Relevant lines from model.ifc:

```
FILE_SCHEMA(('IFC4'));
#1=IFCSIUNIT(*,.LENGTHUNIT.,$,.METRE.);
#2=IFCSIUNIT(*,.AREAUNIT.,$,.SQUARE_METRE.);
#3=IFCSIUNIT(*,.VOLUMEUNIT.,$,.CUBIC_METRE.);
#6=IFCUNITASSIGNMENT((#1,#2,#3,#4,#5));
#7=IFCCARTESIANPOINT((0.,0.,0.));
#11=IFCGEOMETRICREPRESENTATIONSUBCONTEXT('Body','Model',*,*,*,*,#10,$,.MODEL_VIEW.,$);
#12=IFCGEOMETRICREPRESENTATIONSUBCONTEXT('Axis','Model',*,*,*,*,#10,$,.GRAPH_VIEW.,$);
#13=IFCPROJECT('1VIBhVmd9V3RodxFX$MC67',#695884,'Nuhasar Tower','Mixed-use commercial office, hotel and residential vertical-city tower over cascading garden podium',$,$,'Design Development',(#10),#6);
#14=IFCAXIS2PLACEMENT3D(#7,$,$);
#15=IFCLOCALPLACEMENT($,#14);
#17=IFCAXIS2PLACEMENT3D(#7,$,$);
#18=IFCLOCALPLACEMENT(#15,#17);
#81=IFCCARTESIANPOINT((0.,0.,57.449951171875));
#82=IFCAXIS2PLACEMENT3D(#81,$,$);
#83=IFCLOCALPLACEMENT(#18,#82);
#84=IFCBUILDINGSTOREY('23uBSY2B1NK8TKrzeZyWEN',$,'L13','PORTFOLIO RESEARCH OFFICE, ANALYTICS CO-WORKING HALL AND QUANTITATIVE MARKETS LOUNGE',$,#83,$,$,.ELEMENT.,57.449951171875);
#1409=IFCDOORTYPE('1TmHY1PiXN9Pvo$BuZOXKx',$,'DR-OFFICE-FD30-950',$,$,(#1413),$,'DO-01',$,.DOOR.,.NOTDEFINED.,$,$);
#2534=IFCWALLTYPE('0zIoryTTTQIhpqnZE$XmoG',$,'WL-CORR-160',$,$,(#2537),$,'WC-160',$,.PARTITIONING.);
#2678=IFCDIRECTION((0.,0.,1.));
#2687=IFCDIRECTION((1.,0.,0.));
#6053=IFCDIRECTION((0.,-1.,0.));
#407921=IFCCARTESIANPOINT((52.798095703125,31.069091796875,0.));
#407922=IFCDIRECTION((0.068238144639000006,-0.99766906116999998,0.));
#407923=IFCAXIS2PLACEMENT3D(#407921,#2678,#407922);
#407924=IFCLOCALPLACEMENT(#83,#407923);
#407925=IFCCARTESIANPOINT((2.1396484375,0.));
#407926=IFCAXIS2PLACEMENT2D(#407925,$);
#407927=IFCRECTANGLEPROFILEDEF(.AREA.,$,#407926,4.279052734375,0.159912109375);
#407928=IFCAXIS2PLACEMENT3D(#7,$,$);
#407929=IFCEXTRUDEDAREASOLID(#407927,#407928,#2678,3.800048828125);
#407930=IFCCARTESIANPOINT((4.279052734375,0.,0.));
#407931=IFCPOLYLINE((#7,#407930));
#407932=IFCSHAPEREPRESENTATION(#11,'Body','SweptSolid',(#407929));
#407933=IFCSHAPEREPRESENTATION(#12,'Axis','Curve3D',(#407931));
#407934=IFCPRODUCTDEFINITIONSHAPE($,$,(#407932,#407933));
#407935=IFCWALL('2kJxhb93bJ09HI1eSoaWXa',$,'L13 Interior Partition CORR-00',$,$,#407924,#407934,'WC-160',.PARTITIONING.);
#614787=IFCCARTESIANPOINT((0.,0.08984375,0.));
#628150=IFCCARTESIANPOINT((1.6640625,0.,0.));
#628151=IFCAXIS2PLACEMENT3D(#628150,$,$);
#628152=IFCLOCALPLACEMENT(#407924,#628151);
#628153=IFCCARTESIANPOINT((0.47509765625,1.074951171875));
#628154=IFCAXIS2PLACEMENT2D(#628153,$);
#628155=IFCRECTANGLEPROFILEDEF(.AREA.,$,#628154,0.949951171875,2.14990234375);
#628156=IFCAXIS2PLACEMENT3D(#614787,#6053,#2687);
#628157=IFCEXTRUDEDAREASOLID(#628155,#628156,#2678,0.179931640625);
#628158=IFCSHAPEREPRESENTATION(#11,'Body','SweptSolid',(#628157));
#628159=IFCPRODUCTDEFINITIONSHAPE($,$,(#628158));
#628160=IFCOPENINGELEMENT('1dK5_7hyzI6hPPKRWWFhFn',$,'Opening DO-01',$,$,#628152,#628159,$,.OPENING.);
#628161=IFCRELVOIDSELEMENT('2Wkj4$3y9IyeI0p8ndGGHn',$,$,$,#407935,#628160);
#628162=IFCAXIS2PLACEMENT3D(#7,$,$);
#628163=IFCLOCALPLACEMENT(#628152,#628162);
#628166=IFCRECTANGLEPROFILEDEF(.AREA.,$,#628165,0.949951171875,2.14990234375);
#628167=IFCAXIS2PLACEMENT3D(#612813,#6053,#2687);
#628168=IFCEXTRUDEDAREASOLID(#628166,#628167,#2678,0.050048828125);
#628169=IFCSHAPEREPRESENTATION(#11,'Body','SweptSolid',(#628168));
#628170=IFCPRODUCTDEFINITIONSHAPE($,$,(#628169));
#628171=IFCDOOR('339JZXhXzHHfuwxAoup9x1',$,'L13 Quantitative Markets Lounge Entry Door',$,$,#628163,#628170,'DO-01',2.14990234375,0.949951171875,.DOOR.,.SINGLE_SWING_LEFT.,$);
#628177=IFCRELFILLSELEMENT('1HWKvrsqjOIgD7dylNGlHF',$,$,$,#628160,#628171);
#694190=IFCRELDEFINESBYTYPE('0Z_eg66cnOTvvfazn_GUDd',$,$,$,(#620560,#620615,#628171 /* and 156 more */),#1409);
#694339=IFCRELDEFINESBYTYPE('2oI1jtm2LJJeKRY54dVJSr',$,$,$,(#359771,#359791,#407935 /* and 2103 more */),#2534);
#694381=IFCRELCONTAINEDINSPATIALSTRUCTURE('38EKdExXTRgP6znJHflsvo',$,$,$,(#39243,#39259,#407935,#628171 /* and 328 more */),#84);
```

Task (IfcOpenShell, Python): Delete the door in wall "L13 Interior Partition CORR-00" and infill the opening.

```python
import ifcopenshell
import ifcopenshell.api.feature
import ifcopenshell.api.root
import ifcopenshell.geom
import ifcopenshell.util.shape

model = ifcopenshell.open("model.ifc")
settings = ifcopenshell.geom.settings()


def volume(element):
    """Net volume in cubic metres, openings subtracted."""
    shape = ifcopenshell.geom.create_shape(settings, element)
    return ifcopenshell.util.shape.get_volume(shape.geometry)


door = model.by_guid("339JZXhXzHHfuwxAoup9x1")
opening = door.FillsVoids[0].RelatingOpeningElement
wall = opening.VoidsElements[0].RelatingBuildingElement
before = volume(wall)

ifcopenshell.api.root.remove_product(model, product=door)
ifcopenshell.api.feature.remove_feature(model, feature=opening)

after = volume(wall)

print(f"wall volume {before:.3f} -> {after:.3f} m3")

model.write("model_edited.ifc")
```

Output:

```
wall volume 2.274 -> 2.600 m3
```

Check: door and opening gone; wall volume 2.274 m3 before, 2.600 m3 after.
